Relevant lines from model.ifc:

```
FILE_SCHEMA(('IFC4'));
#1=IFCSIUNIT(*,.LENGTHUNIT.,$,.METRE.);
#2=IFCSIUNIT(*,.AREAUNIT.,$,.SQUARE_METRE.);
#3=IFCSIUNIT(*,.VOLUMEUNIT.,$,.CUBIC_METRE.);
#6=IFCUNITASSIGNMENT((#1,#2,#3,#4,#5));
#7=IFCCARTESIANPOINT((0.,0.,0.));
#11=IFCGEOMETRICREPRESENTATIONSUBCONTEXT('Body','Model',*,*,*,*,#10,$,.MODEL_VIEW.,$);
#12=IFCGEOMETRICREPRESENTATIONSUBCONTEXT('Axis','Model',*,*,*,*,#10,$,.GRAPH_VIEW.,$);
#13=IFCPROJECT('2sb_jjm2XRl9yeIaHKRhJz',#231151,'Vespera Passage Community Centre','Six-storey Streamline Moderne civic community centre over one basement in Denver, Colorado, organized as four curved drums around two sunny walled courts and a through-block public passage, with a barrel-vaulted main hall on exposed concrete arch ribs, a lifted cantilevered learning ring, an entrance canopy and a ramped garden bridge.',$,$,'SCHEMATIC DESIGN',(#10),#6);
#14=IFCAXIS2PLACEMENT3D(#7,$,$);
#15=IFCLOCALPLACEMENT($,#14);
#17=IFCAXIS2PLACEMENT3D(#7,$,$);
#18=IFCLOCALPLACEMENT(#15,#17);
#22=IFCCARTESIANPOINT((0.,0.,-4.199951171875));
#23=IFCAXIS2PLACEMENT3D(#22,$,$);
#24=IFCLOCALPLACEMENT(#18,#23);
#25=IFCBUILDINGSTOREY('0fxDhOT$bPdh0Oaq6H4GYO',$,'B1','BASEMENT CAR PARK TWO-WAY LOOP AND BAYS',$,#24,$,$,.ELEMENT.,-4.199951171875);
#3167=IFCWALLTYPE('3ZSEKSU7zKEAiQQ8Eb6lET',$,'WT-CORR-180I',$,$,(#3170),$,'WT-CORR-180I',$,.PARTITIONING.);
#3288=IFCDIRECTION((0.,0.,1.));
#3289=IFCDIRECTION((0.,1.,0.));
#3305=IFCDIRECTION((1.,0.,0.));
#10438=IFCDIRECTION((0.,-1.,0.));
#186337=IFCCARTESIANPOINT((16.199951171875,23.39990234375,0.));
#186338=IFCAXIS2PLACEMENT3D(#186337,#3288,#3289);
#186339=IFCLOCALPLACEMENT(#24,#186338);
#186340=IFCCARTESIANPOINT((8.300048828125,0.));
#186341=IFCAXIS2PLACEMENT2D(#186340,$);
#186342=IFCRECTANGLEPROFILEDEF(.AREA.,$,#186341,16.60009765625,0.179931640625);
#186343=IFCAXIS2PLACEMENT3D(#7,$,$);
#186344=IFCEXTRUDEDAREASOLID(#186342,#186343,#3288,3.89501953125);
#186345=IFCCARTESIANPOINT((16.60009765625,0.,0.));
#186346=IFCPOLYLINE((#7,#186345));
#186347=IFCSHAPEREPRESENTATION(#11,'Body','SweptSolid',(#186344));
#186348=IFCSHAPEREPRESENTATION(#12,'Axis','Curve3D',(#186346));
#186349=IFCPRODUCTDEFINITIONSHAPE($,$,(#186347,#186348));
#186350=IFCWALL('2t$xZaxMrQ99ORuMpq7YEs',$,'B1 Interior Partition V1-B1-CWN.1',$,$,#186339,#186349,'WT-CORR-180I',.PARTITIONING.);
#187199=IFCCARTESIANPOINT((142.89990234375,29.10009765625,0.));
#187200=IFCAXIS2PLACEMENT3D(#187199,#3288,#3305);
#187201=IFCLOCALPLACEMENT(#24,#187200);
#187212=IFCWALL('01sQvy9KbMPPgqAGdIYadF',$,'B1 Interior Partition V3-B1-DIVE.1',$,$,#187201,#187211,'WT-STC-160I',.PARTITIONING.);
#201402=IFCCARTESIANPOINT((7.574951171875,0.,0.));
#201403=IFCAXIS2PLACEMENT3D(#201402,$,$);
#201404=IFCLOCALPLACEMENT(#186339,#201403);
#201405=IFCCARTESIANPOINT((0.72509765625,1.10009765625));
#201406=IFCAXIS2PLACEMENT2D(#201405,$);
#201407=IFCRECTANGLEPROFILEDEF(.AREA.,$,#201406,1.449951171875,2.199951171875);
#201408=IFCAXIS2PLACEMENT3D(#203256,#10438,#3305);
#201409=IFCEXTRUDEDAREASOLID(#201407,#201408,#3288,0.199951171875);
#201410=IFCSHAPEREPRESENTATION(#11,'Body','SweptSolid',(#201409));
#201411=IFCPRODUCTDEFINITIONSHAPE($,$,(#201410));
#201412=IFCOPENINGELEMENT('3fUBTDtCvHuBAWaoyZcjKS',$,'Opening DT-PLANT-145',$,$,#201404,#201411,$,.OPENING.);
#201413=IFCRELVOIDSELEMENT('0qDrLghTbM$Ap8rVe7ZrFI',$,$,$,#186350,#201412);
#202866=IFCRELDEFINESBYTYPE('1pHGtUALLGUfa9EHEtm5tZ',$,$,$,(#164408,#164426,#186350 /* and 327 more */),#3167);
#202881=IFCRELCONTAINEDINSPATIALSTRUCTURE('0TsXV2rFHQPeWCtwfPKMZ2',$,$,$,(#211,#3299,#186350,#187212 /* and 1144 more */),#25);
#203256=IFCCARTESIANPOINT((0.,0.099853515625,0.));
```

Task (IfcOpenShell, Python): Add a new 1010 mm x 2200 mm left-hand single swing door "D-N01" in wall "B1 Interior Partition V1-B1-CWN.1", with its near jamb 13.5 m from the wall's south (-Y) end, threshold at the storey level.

```python
import numpy as np
import ifcopenshell
import ifcopenshell.api.feature
import ifcopenshell.api.geometry
import ifcopenshell.api.root
import ifcopenshell.api.spatial
import ifcopenshell.geom
import ifcopenshell.util.element
import ifcopenshell.util.placement
import ifcopenshell.util.representation
import ifcopenshell.util.shape
import ifcopenshell.util.unit

model = ifcopenshell.open("model.ifc")
unit_scale = ifcopenshell.util.unit.calculate_unit_scale(model)
settings = ifcopenshell.geom.settings()


def volume(element):
    """Net volume in cubic metres, openings subtracted."""
    shape = ifcopenshell.geom.create_shape(settings, element)
    return ifcopenshell.util.shape.get_volume(shape.geometry)


wall = model.by_guid("2t$xZaxMrQ99ORuMpq7YEs")
storey = ifcopenshell.util.element.get_container(wall, ifc_class="IfcBuildingStorey")
context = ifcopenshell.util.representation.get_context(model, "Model", "Body", "MODEL_VIEW")
before = volume(wall)

width, height, from_end, sill = 1.01, 2.2, 13.5, 0.0  # metres

# The wall runs along its own X axis, and the end named is its -X end.
wall_shape = ifcopenshell.geom.create_shape(settings, wall)
x, y, z = ifcopenshell.util.shape.get_vertices(wall_shape.geometry).T
start = x.min() + from_end
face, thickness = float(y.min()), float(y.max() - y.min())
wall_matrix = ifcopenshell.util.placement.get_local_placement(wall.ObjectPlacement)
level = ifcopenshell.util.placement.get_local_placement(storey.ObjectPlacement)[2, 3]


def in_wall(x, y):
    """Placement at x, y metres in the wall's axes, at sill height."""
    matrix = wall_matrix.copy()
    matrix[:, 3] = wall_matrix @ np.array([x / unit_scale, y / unit_scale, 0.0, 1.0])
    matrix[2, 3] = level + sill / unit_scale
    return matrix


# Opening: a box that overshoots both wall faces by 50 mm.
opening = ifcopenshell.api.root.create_entity(model, ifc_class="IfcOpeningElement", predefined_type="OPENING")
box = ifcopenshell.api.geometry.add_wall_representation(
    model, context=context, length=width, height=height, thickness=thickness + 0.1
)
ifcopenshell.api.geometry.assign_representation(model, product=opening, representation=box)
ifcopenshell.api.geometry.edit_object_placement(model, product=opening, matrix=in_wall(start, face - 0.05), is_si=False)
ifcopenshell.api.feature.add_feature(model, feature=opening, element=wall)

door = ifcopenshell.api.root.create_entity(model, ifc_class="IfcDoor", name="D-N01", predefined_type="DOOR")
door.OverallWidth, door.OverallHeight = width / unit_scale, height / unit_scale
door.OperationType = "SINGLE_SWING_LEFT"
body = ifcopenshell.api.geometry.add_door_representation(
    model,
    context=context,
    overall_width=door.OverallWidth,
    overall_height=door.OverallHeight,
    operation_type="SINGLE_SWING_LEFT",
    lining_properties={"LiningDepth": thickness / unit_scale, "ThresholdDepth": thickness / unit_scale},
)
ifcopenshell.api.geometry.assign_representation(model, product=door, representation=body)
ifcopenshell.api.spatial.assign_container(model, products=[door], relating_structure=storey)
ifcopenshell.api.feature.add_filling(model, opening=opening, element=door)

# The lining spans the wall, so the door starts at the wall face.
ifcopenshell.api.geometry.edit_object_placement(model, product=door, matrix=in_wall(start, face), is_si=False)

after = volume(wall)

print(f"wall volume {before:.3f} -> {after:.3f} m3")

model.write("model_edited.ifc")
```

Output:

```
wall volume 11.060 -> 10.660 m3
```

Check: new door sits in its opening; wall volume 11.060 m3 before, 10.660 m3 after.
